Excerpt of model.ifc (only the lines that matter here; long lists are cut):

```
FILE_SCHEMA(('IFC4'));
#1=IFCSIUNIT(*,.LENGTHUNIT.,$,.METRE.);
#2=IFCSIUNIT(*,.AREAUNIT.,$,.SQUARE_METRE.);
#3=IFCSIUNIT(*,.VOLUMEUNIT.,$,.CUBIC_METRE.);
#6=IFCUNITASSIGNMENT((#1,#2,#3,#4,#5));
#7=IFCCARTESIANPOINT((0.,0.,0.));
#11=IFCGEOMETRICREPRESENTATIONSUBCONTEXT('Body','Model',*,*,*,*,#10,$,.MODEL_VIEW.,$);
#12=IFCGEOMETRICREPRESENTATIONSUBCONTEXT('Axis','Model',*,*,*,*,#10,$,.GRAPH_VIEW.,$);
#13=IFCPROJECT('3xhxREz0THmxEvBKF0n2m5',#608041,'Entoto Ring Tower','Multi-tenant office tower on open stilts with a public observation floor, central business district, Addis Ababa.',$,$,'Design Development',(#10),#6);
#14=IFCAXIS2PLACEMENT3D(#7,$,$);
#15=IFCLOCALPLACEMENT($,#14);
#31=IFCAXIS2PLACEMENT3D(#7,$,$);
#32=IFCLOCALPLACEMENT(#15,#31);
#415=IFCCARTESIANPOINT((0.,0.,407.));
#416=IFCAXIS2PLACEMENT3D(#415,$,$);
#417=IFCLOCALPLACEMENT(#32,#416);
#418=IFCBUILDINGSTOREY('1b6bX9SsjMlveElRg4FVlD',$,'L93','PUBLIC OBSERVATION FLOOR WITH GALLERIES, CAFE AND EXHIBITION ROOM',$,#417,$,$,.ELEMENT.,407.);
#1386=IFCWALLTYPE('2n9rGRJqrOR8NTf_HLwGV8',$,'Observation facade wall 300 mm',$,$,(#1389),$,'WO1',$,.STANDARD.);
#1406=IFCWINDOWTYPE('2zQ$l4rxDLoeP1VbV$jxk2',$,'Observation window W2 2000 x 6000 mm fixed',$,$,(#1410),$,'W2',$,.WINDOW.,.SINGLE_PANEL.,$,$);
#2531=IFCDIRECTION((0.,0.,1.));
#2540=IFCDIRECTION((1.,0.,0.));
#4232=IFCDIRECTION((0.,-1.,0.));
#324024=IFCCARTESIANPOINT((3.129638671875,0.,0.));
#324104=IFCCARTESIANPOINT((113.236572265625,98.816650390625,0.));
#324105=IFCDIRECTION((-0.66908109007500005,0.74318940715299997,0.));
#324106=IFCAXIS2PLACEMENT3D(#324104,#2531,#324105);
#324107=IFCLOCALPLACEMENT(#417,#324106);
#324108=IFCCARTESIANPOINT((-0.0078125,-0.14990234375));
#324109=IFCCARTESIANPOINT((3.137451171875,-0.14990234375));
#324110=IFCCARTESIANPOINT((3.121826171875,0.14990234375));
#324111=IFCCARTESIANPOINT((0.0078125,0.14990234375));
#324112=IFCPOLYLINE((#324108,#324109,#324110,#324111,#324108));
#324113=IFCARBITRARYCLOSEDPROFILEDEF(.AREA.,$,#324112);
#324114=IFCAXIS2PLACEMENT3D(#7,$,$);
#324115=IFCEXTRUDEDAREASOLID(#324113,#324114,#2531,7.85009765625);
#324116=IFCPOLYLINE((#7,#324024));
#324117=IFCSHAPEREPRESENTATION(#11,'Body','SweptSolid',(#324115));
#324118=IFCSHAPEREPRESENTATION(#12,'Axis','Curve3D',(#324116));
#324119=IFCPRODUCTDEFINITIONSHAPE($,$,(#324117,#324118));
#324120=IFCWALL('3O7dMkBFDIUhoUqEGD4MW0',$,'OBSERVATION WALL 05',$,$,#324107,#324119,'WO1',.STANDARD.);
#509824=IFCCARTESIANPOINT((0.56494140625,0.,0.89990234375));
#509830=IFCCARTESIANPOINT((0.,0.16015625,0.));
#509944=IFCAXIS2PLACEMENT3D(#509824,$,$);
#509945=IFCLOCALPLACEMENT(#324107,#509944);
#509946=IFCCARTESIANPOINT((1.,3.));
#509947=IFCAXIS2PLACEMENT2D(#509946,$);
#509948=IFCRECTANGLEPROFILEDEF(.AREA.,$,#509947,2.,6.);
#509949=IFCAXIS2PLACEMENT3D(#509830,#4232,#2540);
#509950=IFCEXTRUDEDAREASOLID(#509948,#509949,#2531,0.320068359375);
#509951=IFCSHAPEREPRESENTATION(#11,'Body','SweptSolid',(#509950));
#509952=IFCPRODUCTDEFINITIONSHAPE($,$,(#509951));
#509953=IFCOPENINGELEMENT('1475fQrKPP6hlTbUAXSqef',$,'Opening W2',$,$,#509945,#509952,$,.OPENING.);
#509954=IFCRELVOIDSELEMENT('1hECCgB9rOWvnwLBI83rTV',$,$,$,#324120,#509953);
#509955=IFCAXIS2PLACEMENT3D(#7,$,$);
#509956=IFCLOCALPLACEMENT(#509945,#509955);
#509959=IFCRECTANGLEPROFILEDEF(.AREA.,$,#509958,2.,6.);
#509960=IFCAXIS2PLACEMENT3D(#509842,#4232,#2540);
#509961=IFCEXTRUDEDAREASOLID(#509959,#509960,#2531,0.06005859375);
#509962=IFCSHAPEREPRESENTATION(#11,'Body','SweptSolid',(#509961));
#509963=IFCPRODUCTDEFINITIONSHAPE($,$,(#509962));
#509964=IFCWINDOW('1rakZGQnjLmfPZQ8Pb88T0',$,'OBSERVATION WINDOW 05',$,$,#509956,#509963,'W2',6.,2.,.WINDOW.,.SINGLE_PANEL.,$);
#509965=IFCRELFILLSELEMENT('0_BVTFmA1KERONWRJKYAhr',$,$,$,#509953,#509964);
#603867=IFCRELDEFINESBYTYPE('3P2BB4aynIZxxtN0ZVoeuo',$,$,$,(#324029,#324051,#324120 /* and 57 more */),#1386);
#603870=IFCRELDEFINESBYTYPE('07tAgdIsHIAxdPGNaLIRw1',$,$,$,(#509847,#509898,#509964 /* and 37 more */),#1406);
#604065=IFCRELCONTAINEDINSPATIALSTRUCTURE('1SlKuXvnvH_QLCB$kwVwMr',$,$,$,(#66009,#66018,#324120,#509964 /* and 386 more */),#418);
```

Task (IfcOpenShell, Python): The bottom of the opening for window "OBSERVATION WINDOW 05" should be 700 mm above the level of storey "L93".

```python
import numpy as np
import ifcopenshell
import ifcopenshell.api.geometry
import ifcopenshell.geom
import ifcopenshell.util.element
import ifcopenshell.util.placement
import ifcopenshell.util.shape
import ifcopenshell.util.unit

model = ifcopenshell.open("model.ifc")
unit_scale = ifcopenshell.util.unit.calculate_unit_scale(model)

window = model.by_guid("1rakZGQnjLmfPZQ8Pb88T0")
opening = window.FillsVoids[0].RelatingOpeningElement
storey = ifcopenshell.util.element.get_container(window, ifc_class="IfcBuildingStorey")
level = ifcopenshell.util.placement.get_local_placement(storey.ObjectPlacement)[2, 3]

# The opening's origin need not be at the sill, so measure its lowest point.
shape = ifcopenshell.geom.create_shape(ifcopenshell.geom.settings(), opening)
bottom = ifcopenshell.util.shape.get_shape_bottom_elevation(shape, shape.geometry) / unit_scale
dz = level + 0.7 / unit_scale - bottom

shift = np.array([0.0, 0.0, dz])
# The window is placed relative to its opening, so it follows when the opening moves.
matrix = ifcopenshell.util.placement.get_local_placement(opening.ObjectPlacement)
matrix[:3, 3] += shift
ifcopenshell.api.geometry.edit_object_placement(
    model, product=opening, matrix=matrix, is_si=False, should_transform_children=True
)

print(f"moved by {dz * unit_scale:+.3f} m")

model.write("model_edited.ifc")
```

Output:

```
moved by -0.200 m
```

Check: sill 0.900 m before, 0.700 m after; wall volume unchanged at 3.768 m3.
